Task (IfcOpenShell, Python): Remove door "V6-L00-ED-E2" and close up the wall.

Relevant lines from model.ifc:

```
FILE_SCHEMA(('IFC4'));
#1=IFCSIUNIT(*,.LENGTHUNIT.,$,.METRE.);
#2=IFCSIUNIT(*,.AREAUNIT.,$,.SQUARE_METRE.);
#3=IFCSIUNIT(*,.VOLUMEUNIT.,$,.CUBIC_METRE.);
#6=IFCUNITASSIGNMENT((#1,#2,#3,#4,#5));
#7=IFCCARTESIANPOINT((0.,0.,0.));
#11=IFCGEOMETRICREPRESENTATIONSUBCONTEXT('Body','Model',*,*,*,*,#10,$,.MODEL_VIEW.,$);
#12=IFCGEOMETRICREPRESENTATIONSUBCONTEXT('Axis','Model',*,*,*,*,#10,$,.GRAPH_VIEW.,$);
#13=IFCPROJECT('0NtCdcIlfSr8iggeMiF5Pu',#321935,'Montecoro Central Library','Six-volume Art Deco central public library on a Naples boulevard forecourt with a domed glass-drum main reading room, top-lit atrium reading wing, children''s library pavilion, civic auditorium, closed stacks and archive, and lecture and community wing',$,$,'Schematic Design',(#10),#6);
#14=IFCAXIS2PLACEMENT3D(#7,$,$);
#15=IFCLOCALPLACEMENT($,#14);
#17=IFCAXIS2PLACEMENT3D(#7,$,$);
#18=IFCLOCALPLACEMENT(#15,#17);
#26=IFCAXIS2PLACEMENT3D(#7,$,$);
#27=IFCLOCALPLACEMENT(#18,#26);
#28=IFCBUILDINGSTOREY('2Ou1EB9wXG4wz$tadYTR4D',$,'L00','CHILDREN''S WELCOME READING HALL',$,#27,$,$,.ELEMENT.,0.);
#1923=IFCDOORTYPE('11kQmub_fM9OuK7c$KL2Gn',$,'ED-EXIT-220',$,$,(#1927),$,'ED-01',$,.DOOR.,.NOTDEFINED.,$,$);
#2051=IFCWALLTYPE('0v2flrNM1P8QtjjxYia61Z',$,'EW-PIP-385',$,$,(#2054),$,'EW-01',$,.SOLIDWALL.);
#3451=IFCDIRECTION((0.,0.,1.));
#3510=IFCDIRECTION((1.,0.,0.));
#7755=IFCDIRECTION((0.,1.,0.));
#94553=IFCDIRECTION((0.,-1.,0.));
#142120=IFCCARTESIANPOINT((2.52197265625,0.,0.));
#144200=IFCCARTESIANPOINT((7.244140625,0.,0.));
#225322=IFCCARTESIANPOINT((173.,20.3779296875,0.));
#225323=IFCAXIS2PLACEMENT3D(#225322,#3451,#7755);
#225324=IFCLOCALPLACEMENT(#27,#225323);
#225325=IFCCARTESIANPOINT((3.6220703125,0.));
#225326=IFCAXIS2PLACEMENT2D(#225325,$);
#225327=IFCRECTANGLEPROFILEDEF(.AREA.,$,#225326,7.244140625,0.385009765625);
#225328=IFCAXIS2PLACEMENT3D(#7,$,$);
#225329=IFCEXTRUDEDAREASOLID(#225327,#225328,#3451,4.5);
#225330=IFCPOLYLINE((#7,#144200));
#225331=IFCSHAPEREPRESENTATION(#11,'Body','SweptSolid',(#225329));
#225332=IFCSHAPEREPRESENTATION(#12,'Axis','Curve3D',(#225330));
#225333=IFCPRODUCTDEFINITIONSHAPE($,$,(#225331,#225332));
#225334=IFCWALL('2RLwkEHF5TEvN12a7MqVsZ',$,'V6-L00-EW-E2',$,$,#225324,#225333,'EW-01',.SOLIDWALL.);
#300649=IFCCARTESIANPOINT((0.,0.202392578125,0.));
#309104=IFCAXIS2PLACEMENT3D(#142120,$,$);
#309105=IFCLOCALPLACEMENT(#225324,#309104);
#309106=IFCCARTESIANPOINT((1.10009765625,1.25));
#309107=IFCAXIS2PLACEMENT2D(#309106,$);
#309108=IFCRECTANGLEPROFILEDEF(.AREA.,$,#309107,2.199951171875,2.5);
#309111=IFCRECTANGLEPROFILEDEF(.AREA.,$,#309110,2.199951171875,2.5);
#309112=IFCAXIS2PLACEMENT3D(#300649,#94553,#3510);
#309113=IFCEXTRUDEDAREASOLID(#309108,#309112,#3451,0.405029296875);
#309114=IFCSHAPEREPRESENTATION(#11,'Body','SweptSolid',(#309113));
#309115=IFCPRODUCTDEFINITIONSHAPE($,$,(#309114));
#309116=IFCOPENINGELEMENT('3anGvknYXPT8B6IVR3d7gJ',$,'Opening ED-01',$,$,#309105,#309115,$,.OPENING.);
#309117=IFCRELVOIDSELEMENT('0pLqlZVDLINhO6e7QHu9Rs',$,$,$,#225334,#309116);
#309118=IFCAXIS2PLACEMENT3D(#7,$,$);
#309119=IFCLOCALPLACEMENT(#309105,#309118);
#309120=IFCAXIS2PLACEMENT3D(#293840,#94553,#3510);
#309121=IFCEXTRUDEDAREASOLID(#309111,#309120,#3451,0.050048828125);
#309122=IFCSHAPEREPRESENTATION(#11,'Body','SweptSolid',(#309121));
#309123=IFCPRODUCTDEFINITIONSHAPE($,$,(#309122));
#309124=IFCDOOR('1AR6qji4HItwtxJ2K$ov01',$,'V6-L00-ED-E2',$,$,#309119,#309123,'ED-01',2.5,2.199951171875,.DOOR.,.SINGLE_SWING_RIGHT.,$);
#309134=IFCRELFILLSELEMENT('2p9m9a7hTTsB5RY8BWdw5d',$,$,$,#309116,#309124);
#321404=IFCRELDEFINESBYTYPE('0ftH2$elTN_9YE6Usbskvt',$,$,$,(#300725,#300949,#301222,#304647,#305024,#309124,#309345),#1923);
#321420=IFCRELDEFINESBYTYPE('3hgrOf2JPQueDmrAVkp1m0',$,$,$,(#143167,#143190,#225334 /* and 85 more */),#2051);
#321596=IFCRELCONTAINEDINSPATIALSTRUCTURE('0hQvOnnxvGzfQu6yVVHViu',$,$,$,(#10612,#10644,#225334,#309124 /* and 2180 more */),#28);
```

```python
import ifcopenshell
import ifcopenshell.api.feature
import ifcopenshell.api.root
import ifcopenshell.geom
import ifcopenshell.util.shape

model = ifcopenshell.open("model.ifc")
settings = ifcopenshell.geom.settings()


def volume(element):
    """Net volume in cubic metres, openings subtracted."""
    shape = ifcopenshell.geom.create_shape(settings, element)
    return ifcopenshell.util.shape.get_volume(shape.geometry)


door = model.by_guid("1AR6qji4HItwtxJ2K$ov01")
opening = door.FillsVoids[0].RelatingOpeningElement
wall = opening.VoidsElements[0].RelatingBuildingElement
before = volume(wall)

ifcopenshell.api.root.remove_product(model, product=door)
ifcopenshell.api.feature.remove_feature(model, feature=opening)

after = volume(wall)

print(f"wall volume {before:.3f} -> {after:.3f} m3")

model.write("model_edited.ifc")
```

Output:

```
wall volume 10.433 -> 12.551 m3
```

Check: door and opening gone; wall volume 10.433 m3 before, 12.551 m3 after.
